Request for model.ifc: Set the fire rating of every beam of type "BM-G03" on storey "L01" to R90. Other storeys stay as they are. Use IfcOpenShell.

First a look at what the model holds.

```python
import ifcopenshell
import ifcopenshell.util.element

model = ifcopenshell.open("model.ifc")
print(model.schema)
storey = next(s for s in model.by_type("IfcBuildingStorey") if s.Name == "L01")
beams = [e for e in ifcopenshell.util.element.get_decomposition(storey) if e.is_a("IfcBeam")]
seen = {}
for e in beams:
    element_type = ifcopenshell.util.element.get_type(e)
    key = (element_type.Name if element_type != e and element_type else None, ifcopenshell.util.element.get_pset(e, "Pset_BeamCommon", "FireRating"))
    seen[key] = seen.get(key, 0) + 1
for (name, value), count in sorted(seen.items(), key=str):
    print(count, "x", name, "|", value)
```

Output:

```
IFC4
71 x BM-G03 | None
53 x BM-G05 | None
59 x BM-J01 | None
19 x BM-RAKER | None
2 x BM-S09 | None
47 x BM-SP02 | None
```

```python
import ifcopenshell
import ifcopenshell.api.pset
import ifcopenshell.util.element

model = ifcopenshell.open("model.ifc")

storey = next(s for s in model.by_type("IfcBuildingStorey") if s.Name == "L01")
beams = [e for e in ifcopenshell.util.element.get_decomposition(storey) if e.is_a("IfcBeam")]

count = 0
for e in beams:
    element_type = ifcopenshell.util.element.get_type(e)
    if element_type in (None, e) or element_type.Name != "BM-G03":
        continue
    # add_pset returns the element's existing set when there is one.
    pset = ifcopenshell.api.pset.add_pset(model, product=e, name="Pset_BeamCommon")
    ifcopenshell.api.pset.edit_pset(model, pset=pset, properties={"FireRating": "R90"})
    count += 1

print(count, "beams updated")

model.write("model_updated.ifc")
```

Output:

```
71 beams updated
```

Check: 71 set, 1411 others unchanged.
